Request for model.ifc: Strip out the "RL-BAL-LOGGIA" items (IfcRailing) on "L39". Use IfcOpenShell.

First a look at what the model holds.

```python
import ifcopenshell
import ifcopenshell.util.element

model = ifcopenshell.open("model.ifc")
print(model.schema)
storey = next(s for s in model.by_type("IfcBuildingStorey") if s.Name == "L39")
railings = [e for e in ifcopenshell.util.element.get_decomposition(storey) if e.is_a("IfcRailing")]
seen = {}
for e in railings:
    element_type = ifcopenshell.util.element.get_type(e)
    name = element_type.Name if element_type not in (None, e) else None
    seen[name] = seen.get(name, 0) + 1
for name, count in sorted(seen.items(), key=str):
    print(count, "x", name)
```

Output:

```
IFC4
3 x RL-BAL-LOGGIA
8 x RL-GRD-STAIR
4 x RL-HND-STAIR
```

```python
import ifcopenshell
import ifcopenshell.api.root
import ifcopenshell.util.element

model = ifcopenshell.open("model.ifc")

storey = next(s for s in model.by_type("IfcBuildingStorey") if s.Name == "L39")
railings = [e for e in ifcopenshell.util.element.get_decomposition(storey) if e.is_a("IfcRailing")]
targets = [e for e in railings if (t := ifcopenshell.util.element.get_type(e)) not in (None, e) and t.Name == "RL-BAL-LOGGIA"]

for e in targets:
    ifcopenshell.api.root.remove_product(model, product=e)
print(len(targets), "removed")

model.write("model_updated.ifc")
```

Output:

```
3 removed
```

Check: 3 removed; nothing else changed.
